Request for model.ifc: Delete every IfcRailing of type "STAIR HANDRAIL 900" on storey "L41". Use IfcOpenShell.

First a look at what the model holds.

```python
import ifcopenshell
import ifcopenshell.util.element

model = ifcopenshell.open("model.ifc")
print(model.schema)
storey = next(s for s in model.by_type("IfcBuildingStorey") if s.Name == "L41")
railings = [e for e in ifcopenshell.util.element.get_decomposition(storey) if e.is_a("IfcRailing")]
seen = {}
for e in railings:
    element_type = ifcopenshell.util.element.get_type(e)
    name = element_type.Name if element_type not in (None, e) else None
    seen[name] = seen.get(name, 0) + 1
for name, count in sorted(seen.items(), key=str):
    print(count, "x", name)
```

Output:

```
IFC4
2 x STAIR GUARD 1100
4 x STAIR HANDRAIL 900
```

```python
import ifcopenshell
import ifcopenshell.api.root
import ifcopenshell.util.element

model = ifcopenshell.open("model.ifc")

storey = next(s for s in model.by_type("IfcBuildingStorey") if s.Name == "L41")
railings = [e for e in ifcopenshell.util.element.get_decomposition(storey) if e.is_a("IfcRailing")]
targets = [e for e in railings if (t := ifcopenshell.util.element.get_type(e)) not in (None, e) and t.Name == "STAIR HANDRAIL 900"]

for e in targets:
    ifcopenshell.api.root.remove_product(model, product=e)
print(len(targets), "removed")

model.write("model_v2.ifc")
```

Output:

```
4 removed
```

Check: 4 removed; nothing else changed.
